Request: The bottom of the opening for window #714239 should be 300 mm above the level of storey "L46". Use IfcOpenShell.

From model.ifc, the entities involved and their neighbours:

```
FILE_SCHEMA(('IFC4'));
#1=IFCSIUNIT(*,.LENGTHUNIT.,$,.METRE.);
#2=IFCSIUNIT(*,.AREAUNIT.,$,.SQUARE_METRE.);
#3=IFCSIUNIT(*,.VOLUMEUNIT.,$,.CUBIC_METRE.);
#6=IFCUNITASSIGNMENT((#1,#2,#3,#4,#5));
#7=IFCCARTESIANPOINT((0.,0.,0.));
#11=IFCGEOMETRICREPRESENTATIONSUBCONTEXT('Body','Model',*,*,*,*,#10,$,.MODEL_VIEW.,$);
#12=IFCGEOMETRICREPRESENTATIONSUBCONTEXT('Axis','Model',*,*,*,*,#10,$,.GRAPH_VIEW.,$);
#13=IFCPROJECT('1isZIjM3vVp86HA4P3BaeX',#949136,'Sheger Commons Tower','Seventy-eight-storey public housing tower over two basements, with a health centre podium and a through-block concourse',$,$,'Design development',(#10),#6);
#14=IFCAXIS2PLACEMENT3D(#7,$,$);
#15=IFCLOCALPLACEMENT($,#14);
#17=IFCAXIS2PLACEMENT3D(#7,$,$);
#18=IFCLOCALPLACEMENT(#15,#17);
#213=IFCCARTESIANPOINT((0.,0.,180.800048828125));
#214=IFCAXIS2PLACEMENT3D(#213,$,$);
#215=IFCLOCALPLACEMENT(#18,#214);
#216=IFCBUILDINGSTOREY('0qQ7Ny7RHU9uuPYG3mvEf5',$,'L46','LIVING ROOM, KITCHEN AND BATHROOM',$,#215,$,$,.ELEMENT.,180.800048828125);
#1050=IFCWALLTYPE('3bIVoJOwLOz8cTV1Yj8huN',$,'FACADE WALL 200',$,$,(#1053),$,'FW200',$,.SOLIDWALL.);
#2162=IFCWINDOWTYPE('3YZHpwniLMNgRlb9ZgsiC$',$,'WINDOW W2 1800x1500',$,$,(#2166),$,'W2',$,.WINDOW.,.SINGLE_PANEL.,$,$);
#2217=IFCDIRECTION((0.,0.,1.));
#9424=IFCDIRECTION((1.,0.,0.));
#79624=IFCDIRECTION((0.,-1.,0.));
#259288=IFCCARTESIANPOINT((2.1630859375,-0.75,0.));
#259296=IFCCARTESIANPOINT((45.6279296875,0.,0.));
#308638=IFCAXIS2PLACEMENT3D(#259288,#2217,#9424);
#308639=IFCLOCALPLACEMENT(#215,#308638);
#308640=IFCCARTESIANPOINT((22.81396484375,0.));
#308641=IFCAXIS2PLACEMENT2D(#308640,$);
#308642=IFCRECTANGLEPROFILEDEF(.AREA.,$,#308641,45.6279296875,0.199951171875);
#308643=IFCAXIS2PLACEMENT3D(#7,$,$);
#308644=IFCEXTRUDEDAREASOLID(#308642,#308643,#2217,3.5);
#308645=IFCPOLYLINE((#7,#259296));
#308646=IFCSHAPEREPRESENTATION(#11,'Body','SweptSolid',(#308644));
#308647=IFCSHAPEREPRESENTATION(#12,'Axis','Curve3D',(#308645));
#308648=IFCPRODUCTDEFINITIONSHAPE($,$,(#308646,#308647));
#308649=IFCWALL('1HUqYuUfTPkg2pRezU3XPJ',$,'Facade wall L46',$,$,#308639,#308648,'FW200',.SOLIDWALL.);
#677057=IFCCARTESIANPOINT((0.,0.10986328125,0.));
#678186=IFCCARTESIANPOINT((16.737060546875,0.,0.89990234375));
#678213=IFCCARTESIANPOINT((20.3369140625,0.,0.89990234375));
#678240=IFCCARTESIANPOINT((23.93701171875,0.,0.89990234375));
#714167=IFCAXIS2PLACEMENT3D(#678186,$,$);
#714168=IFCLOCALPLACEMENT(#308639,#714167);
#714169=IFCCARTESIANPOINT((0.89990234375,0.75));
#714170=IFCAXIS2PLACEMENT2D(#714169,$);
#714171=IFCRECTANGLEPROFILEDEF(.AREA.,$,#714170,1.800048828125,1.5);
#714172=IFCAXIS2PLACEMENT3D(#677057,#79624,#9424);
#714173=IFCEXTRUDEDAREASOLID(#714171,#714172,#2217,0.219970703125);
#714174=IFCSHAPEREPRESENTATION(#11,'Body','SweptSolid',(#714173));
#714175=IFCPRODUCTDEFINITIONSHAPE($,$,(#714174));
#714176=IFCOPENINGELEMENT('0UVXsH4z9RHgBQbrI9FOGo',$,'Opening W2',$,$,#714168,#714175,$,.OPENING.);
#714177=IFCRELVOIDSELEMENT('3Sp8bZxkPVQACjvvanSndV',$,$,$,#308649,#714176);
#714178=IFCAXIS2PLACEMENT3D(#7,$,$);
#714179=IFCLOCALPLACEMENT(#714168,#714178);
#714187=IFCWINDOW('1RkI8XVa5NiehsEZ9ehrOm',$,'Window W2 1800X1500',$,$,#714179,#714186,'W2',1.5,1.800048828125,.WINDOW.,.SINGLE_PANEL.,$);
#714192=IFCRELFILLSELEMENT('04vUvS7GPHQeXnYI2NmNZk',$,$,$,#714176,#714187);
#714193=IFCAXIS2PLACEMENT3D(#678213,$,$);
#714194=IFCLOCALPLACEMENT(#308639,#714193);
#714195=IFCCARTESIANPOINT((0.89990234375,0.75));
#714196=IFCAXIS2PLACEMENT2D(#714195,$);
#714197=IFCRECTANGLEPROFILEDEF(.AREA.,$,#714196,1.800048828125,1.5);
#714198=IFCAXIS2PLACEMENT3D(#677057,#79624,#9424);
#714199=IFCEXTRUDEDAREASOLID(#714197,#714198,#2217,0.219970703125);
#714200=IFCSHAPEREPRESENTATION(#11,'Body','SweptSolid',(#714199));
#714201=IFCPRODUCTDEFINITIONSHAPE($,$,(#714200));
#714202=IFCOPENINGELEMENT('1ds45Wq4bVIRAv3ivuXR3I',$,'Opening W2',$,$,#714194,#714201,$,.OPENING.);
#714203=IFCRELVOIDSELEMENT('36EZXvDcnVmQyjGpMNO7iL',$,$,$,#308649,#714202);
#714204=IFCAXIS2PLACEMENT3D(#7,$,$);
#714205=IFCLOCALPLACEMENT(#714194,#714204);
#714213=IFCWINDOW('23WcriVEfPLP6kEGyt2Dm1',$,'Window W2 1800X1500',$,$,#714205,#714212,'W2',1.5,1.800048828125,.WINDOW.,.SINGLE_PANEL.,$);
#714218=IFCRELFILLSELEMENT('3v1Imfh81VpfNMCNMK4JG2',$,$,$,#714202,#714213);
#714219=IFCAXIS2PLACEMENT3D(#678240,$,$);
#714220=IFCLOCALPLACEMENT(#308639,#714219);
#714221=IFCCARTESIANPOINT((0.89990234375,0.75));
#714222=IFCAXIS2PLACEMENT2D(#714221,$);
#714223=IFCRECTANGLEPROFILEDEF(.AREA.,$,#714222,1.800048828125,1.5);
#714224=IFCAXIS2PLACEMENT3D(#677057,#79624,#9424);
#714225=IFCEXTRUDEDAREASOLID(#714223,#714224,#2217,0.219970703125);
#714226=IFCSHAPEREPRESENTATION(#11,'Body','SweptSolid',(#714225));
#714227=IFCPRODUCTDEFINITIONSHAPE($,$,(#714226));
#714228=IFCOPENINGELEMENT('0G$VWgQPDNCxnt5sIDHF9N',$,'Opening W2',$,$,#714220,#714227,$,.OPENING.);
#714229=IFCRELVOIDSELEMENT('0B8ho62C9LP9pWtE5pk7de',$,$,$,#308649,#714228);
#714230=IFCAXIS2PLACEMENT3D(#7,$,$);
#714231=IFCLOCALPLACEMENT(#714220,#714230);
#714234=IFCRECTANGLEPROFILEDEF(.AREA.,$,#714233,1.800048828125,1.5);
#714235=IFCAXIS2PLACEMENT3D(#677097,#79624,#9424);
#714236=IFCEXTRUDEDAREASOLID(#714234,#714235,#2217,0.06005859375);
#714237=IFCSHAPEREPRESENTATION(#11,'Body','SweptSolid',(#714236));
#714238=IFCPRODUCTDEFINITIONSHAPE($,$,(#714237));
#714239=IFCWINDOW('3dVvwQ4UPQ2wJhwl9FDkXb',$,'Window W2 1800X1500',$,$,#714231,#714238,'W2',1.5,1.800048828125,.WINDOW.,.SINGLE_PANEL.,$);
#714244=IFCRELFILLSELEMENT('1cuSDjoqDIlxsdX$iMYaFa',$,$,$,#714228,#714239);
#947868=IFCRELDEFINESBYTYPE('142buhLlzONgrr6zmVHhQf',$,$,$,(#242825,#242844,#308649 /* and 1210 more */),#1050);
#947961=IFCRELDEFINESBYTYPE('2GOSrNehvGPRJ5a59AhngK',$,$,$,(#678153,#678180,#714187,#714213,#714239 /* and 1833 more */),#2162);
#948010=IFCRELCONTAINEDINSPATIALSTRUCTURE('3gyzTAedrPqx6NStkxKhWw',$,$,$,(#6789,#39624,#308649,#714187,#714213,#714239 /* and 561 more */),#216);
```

```python
import numpy as np
import ifcopenshell
import ifcopenshell.api.geometry
import ifcopenshell.geom
import ifcopenshell.util.element
import ifcopenshell.util.placement
import ifcopenshell.util.shape
import ifcopenshell.util.unit

model = ifcopenshell.open("model.ifc")
unit_scale = ifcopenshell.util.unit.calculate_unit_scale(model)

window = model.by_id(714239)
opening = window.FillsVoids[0].RelatingOpeningElement
storey = ifcopenshell.util.element.get_container(window, ifc_class="IfcBuildingStorey")
level = ifcopenshell.util.placement.get_local_placement(storey.ObjectPlacement)[2, 3]

# The opening's origin need not be at the sill, so measure its lowest point.
shape = ifcopenshell.geom.create_shape(ifcopenshell.geom.settings(), opening)
bottom = ifcopenshell.util.shape.get_shape_bottom_elevation(shape, shape.geometry) / unit_scale
dz = level + 0.3 / unit_scale - bottom

shift = np.array([0.0, 0.0, dz])
# The window is placed relative to its opening, so it follows when the opening moves.
matrix = ifcopenshell.util.placement.get_local_placement(opening.ObjectPlacement)
matrix[:3, 3] += shift
ifcopenshell.api.geometry.edit_object_placement(
    model, product=opening, matrix=matrix, is_si=False, should_transform_children=True
)

print(f"moved by {dz * unit_scale:+.3f} m")

model.write("model_rev.ifc")
```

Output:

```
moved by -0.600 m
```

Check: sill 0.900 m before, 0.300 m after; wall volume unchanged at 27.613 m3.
